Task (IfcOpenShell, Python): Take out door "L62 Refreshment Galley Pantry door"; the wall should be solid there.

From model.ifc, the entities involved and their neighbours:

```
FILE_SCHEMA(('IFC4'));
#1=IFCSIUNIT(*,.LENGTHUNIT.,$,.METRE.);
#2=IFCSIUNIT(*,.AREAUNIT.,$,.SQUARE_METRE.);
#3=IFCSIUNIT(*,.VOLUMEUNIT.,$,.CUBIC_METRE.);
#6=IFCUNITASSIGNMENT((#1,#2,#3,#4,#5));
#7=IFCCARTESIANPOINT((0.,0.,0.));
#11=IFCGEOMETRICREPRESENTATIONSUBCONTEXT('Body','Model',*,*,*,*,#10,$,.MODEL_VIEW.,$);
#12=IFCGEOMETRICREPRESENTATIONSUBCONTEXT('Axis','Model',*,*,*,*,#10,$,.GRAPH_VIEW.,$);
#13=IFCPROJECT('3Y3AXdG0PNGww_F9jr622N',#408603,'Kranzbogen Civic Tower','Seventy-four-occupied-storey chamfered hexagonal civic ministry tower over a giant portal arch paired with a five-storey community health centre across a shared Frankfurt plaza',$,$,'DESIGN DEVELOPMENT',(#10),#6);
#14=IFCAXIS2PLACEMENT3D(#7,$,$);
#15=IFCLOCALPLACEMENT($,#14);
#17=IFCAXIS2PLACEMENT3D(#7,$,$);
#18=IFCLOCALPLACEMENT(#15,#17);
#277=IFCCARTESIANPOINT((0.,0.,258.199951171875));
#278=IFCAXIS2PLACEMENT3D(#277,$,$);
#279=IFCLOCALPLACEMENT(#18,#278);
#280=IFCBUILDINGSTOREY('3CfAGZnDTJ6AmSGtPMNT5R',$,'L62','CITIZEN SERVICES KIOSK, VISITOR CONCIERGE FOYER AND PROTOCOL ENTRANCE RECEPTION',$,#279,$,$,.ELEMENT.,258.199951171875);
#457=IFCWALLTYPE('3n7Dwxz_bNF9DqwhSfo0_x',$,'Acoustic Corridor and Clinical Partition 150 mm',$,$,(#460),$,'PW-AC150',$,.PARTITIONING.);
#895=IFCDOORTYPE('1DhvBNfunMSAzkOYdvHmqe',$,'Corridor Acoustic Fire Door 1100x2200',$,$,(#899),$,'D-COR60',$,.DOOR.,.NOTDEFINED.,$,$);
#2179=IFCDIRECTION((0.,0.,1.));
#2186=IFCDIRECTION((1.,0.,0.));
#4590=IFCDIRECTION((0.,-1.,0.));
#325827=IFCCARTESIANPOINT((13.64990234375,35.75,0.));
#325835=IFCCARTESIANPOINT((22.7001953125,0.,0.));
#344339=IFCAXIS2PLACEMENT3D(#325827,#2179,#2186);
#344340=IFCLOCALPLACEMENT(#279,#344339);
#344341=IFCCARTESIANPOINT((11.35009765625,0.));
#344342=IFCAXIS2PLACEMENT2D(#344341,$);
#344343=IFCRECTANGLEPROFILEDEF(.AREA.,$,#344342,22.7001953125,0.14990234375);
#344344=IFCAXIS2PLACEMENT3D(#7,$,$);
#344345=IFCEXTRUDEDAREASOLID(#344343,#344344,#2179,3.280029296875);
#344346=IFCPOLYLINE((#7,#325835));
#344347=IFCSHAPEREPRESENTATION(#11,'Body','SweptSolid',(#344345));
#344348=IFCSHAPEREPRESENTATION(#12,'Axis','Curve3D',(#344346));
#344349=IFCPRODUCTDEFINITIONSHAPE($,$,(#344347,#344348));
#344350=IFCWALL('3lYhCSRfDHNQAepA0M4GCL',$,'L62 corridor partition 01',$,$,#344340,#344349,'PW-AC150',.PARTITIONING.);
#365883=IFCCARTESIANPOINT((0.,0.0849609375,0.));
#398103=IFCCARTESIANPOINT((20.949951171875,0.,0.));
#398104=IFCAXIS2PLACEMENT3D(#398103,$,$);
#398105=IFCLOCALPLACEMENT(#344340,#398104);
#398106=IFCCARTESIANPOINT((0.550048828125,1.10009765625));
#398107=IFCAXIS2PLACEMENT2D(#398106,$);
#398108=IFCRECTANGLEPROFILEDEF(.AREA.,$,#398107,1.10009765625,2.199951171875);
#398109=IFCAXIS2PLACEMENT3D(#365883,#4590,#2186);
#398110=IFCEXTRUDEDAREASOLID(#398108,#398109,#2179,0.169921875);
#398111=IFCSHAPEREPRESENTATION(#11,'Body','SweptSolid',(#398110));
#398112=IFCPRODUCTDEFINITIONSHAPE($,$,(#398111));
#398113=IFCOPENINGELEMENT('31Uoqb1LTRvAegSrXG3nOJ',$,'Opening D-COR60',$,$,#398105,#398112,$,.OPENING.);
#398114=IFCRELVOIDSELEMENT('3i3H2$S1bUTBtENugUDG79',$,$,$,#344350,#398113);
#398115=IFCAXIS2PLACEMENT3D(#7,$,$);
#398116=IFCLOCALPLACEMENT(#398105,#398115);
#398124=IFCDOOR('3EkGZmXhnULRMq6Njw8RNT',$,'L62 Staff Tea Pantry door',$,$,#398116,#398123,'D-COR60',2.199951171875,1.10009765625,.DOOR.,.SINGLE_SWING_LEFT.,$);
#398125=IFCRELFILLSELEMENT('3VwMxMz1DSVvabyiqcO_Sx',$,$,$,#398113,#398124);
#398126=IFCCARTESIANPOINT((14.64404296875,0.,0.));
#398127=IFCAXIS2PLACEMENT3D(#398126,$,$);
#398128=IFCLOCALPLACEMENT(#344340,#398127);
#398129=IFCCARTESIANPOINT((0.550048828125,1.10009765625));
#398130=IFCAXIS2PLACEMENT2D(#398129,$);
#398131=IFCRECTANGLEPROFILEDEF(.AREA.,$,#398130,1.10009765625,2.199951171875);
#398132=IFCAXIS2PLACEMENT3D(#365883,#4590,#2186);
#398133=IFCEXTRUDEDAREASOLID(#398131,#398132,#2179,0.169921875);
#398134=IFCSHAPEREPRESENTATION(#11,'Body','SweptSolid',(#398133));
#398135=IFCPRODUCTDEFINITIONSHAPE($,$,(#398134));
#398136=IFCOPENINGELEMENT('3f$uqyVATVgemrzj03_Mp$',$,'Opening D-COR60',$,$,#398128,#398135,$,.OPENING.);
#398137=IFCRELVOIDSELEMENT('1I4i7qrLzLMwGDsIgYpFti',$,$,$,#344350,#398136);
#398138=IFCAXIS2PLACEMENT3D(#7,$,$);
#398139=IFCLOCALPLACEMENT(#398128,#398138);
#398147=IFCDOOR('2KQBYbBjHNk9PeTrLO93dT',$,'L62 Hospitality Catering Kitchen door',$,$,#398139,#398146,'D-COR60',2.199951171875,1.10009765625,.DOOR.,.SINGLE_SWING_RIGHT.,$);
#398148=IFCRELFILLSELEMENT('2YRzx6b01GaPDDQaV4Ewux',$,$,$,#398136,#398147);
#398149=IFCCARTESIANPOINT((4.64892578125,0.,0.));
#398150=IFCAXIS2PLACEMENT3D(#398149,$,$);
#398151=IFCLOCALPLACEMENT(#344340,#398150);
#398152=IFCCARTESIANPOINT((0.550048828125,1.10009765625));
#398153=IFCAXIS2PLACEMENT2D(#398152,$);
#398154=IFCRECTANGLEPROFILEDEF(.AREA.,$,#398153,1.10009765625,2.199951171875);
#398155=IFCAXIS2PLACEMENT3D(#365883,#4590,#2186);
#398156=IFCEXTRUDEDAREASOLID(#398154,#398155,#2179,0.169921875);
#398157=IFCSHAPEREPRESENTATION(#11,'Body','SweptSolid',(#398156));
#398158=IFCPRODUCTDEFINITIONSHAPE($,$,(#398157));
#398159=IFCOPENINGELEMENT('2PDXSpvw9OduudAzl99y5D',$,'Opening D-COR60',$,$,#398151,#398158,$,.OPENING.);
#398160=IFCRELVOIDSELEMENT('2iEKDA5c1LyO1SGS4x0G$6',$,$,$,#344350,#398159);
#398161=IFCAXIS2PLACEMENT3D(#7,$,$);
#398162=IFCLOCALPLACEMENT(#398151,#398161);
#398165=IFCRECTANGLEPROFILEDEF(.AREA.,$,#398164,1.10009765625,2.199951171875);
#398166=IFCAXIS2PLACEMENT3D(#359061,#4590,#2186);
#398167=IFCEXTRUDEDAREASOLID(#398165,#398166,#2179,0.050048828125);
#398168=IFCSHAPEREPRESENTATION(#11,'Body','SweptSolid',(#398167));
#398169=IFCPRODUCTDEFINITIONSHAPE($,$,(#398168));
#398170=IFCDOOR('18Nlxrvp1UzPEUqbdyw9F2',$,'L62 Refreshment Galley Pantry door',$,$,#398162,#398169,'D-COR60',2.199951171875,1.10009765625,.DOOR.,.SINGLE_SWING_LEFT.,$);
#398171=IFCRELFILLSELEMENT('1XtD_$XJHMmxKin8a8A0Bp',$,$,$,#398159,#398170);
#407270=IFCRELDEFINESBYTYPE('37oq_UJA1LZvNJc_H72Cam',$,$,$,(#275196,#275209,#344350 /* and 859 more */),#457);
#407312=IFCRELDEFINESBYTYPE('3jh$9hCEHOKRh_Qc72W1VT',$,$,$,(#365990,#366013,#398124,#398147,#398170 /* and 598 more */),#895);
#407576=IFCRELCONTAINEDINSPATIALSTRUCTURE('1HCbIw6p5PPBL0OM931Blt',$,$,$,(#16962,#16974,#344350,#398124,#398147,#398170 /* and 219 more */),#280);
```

```python
import ifcopenshell
import ifcopenshell.api.feature
import ifcopenshell.api.root
import ifcopenshell.geom
import ifcopenshell.util.shape

model = ifcopenshell.open("model.ifc")
settings = ifcopenshell.geom.settings()


def volume(element):
    """Net volume in cubic metres, openings subtracted."""
    shape = ifcopenshell.geom.create_shape(settings, element)
    return ifcopenshell.util.shape.get_volume(shape.geometry)


door = model.by_id(398170)
opening = door.FillsVoids[0].RelatingOpeningElement
wall = opening.VoidsElements[0].RelatingBuildingElement
before = volume(wall)

ifcopenshell.api.root.remove_product(model, product=door)
ifcopenshell.api.feature.remove_feature(model, feature=opening)

after = volume(wall)

print(f"wall volume {before:.3f} -> {after:.3f} m3")

model.write("model_rev.ifc")
```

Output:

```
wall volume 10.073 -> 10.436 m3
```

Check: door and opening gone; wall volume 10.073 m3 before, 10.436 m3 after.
